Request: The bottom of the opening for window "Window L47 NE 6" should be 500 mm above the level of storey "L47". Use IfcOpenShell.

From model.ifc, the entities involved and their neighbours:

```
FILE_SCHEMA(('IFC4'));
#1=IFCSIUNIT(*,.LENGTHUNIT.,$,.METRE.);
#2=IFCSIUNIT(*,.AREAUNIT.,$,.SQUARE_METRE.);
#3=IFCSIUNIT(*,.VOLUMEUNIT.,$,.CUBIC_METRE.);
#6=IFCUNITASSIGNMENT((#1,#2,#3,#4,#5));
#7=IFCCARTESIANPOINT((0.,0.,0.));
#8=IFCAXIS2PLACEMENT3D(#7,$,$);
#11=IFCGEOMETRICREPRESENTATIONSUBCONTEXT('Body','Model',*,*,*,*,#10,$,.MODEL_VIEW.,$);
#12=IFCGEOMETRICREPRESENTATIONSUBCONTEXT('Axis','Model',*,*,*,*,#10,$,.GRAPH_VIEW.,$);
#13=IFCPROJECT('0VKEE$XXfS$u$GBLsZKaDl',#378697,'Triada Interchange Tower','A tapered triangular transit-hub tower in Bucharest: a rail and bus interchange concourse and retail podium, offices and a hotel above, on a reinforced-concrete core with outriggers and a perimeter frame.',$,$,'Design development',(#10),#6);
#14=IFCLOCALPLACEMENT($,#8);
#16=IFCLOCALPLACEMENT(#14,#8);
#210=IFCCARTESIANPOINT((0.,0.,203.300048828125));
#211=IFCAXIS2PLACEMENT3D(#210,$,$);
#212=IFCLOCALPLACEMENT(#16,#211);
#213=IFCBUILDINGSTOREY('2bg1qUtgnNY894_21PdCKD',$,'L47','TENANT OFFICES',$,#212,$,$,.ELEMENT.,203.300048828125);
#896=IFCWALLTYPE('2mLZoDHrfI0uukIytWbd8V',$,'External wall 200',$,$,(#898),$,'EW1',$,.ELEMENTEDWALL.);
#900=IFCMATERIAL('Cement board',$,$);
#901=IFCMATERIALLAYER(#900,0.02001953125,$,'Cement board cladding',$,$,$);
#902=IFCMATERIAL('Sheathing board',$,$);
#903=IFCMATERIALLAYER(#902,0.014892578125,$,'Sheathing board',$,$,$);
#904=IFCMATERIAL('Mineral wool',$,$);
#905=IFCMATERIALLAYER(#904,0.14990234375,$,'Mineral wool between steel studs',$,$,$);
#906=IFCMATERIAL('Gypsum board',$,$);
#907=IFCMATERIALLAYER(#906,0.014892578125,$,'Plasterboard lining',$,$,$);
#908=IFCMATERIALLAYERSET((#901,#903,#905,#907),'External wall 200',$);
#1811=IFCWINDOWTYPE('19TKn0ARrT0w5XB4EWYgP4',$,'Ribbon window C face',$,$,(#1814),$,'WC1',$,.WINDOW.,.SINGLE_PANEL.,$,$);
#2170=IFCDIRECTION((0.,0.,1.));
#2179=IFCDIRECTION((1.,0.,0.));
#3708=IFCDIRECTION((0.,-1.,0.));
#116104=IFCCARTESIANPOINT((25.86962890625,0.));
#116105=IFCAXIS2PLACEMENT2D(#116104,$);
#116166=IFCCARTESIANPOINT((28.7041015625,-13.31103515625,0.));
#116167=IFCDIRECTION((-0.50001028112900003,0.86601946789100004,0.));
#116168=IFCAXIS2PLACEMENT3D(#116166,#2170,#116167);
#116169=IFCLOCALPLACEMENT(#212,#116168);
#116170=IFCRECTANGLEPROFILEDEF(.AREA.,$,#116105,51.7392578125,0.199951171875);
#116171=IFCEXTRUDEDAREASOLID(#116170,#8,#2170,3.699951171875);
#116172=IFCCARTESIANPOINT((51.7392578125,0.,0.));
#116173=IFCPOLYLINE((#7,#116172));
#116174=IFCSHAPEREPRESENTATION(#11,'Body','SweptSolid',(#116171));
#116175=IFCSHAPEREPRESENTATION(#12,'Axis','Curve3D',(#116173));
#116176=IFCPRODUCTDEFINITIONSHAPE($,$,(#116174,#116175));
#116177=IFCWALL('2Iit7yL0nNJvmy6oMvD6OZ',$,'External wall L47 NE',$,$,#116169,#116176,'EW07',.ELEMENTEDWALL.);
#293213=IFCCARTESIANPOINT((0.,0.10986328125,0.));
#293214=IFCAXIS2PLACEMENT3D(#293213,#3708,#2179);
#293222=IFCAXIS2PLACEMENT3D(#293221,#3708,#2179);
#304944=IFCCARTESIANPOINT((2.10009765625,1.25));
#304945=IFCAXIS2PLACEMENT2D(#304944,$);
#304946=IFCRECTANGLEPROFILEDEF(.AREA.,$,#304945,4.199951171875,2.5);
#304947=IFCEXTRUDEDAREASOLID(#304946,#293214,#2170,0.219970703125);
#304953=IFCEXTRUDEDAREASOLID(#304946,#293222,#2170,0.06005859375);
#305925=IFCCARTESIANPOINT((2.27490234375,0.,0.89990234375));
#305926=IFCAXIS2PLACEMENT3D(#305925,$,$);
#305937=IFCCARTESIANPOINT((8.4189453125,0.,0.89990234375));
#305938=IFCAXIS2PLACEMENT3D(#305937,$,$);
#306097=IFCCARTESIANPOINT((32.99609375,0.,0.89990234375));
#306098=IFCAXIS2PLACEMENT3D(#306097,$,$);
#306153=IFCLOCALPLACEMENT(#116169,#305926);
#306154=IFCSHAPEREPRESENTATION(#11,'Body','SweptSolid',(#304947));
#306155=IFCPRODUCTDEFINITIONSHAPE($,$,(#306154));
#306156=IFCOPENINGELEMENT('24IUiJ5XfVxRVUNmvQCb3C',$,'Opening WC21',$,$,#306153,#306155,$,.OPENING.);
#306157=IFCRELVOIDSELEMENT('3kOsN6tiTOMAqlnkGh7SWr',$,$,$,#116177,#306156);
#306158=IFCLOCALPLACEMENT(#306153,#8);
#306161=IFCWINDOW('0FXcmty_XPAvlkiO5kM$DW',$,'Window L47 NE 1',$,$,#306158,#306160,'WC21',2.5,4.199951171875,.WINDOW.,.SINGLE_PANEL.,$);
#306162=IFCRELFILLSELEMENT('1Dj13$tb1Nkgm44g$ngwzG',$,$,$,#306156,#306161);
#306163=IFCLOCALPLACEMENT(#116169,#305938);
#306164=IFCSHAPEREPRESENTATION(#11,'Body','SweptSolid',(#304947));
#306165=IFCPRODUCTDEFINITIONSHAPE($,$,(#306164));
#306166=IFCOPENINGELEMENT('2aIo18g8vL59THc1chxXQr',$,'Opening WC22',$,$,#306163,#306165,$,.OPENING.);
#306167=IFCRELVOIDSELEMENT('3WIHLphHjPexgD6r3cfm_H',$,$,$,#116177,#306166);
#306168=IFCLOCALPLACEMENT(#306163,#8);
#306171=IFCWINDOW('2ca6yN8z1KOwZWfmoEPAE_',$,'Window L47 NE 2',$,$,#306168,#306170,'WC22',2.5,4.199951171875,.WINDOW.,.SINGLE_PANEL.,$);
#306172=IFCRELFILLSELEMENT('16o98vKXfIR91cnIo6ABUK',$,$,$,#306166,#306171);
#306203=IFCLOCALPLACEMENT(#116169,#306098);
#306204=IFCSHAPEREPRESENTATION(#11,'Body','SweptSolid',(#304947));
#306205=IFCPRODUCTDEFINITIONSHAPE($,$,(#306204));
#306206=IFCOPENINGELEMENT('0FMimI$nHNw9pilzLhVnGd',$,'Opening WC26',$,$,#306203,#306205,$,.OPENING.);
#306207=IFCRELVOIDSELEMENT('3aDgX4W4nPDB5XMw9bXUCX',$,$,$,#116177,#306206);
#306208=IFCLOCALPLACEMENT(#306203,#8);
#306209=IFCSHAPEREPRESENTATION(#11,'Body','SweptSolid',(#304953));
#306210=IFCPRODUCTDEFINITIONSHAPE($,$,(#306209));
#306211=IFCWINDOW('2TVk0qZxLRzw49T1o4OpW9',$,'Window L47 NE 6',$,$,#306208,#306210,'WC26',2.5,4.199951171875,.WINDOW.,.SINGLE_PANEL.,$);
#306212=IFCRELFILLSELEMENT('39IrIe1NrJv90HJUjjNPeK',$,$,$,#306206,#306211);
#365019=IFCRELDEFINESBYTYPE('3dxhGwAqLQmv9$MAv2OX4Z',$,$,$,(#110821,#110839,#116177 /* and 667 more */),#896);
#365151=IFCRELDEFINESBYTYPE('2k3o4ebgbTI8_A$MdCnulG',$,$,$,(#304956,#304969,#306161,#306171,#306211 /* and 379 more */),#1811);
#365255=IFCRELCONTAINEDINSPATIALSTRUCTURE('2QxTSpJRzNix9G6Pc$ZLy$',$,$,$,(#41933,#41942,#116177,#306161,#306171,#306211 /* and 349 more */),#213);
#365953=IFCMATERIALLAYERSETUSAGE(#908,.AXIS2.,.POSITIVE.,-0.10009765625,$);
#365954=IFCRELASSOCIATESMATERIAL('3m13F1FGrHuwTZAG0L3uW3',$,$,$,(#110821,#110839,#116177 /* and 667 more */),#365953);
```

```python
import numpy as np
import ifcopenshell
import ifcopenshell.api.geometry
import ifcopenshell.geom
import ifcopenshell.util.element
import ifcopenshell.util.placement
import ifcopenshell.util.shape
import ifcopenshell.util.unit

model = ifcopenshell.open("model.ifc")
unit_scale = ifcopenshell.util.unit.calculate_unit_scale(model)

window = model.by_guid("2TVk0qZxLRzw49T1o4OpW9")
opening = window.FillsVoids[0].RelatingOpeningElement
storey = ifcopenshell.util.element.get_container(window, ifc_class="IfcBuildingStorey")
level = ifcopenshell.util.placement.get_local_placement(storey.ObjectPlacement)[2, 3]

# The opening's origin need not be at the sill, so measure its lowest point.
shape = ifcopenshell.geom.create_shape(ifcopenshell.geom.settings(), opening)
bottom = ifcopenshell.util.shape.get_shape_bottom_elevation(shape, shape.geometry) / unit_scale
dz = level + 0.5 - bottom

shift = np.array([0.0, 0.0, dz])
# The window is placed relative to its opening, so it follows when the opening moves.
matrix = ifcopenshell.util.placement.get_local_placement(opening.ObjectPlacement)
matrix[:3, 3] += shift
ifcopenshell.api.geometry.edit_object_placement(
    model, product=opening, matrix=matrix, is_si=False, should_transform_children=True
)

print(f"moved by {dz * unit_scale:+.3f} m")

model.write("model_edited.ifc")
```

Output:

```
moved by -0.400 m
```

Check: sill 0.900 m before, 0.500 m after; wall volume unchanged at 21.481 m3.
